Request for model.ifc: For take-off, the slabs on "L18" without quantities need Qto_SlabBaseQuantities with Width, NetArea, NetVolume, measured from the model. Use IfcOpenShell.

First a look at what the model holds.

```python
import ifcopenshell
import ifcopenshell.util.element
import ifcopenshell.util.unit

model = ifcopenshell.open("model.ifc")
print(model.schema)
for unit_type in ("LENGTHUNIT", "AREAUNIT", "VOLUMEUNIT"):
    print(unit_type, ifcopenshell.util.unit.calculate_unit_scale(model, unit_type))
storey = next(s for s in model.by_type("IfcBuildingStorey") if s.Name == "L18")
slabs = [e for e in ifcopenshell.util.element.get_decomposition(storey) if e.is_a("IfcSlab")]
for e in sorted(slabs, key=lambda e: e.id()):
    print(e.id(), e.is_a(), e.Name, list(ifcopenshell.util.element.get_psets(e, qtos_only=True)), sep=" | ")
```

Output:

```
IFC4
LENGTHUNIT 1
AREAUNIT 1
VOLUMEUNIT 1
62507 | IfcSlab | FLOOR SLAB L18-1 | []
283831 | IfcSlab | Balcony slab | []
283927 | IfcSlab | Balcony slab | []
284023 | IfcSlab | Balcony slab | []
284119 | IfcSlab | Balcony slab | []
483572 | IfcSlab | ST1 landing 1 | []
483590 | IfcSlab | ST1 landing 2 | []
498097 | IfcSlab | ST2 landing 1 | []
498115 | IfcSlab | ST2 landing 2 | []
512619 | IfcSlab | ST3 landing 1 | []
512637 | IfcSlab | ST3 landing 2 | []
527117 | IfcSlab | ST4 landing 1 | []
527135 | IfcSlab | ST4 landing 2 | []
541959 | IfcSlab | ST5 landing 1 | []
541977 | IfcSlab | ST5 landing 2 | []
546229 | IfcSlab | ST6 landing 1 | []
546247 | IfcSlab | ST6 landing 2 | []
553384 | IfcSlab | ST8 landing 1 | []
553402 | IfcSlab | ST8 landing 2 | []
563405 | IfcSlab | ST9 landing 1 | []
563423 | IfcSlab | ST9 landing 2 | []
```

```python
import ifcopenshell
import ifcopenshell.api.pset
import ifcopenshell.geom
import ifcopenshell.util.element
import ifcopenshell.util.shape
import ifcopenshell.util.unit

model = ifcopenshell.open("model.ifc")
unit_scale = ifcopenshell.util.unit.calculate_unit_scale(model)
area_scale = ifcopenshell.util.unit.calculate_unit_scale(model, "AREAUNIT")
volume_scale = ifcopenshell.util.unit.calculate_unit_scale(model, "VOLUMEUNIT")
settings = ifcopenshell.geom.settings()

storey = next(s for s in model.by_type("IfcBuildingStorey") if s.Name == "L18")
slabs = [e for e in ifcopenshell.util.element.get_decomposition(storey) if e.is_a("IfcSlab")]

for e in sorted(slabs, key=lambda e: e.id()):
    if ifcopenshell.util.element.get_psets(e, qtos_only=True, should_inherit=False):
        continue
    # Geometry comes back in metres, in the element's own axes.
    shape = ifcopenshell.geom.create_shape(settings, e)
    values = {
        "Width": ifcopenshell.util.shape.get_z(shape.geometry) / unit_scale,
        "NetArea": ifcopenshell.util.shape.get_footprint_area(shape.geometry) / area_scale,
        "NetVolume": ifcopenshell.util.shape.get_volume(shape.geometry) / volume_scale,
    }
    qto = ifcopenshell.api.pset.add_qto(model, product=e, name="Qto_SlabBaseQuantities")
    ifcopenshell.api.pset.edit_qto(model, qto=qto, properties=values)
    print(e.id(), {k: round(v, 3) for k, v in values.items()})

model.write("model_rev.ifc")
```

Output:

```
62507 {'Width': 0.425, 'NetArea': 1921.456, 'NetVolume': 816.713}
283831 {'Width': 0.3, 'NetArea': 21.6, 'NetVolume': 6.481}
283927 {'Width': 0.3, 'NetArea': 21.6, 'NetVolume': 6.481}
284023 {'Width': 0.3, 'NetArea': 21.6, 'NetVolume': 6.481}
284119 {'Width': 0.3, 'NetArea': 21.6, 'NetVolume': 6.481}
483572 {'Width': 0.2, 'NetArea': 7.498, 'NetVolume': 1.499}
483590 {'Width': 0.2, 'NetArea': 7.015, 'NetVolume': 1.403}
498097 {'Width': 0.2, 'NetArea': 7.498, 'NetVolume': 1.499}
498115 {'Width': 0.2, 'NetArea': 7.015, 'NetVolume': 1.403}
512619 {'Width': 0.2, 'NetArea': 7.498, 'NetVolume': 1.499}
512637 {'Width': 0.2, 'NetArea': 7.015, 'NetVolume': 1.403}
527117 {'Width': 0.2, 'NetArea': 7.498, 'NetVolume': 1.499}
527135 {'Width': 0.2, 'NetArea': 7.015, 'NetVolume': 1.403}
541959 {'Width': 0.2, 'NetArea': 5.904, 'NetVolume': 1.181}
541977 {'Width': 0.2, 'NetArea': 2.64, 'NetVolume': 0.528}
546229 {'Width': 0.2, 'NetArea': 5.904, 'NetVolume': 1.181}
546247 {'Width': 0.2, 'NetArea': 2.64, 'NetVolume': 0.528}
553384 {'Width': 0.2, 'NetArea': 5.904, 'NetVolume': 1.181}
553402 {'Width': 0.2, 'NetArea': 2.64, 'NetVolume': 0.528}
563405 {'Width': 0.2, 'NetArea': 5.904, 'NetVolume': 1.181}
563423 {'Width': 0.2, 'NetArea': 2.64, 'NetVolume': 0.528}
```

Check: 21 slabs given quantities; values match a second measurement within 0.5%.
